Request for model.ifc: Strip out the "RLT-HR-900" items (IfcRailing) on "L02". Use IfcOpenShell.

First a look at what the model holds.

```python
import ifcopenshell
import ifcopenshell.util.element

model = ifcopenshell.open("model.ifc")
print(model.schema)
storey = next(s for s in model.by_type("IfcBuildingStorey") if s.Name == "L02")
railings = [e for e in ifcopenshell.util.element.get_decomposition(storey) if e.is_a("IfcRailing")]
seen = {}
for e in railings:
    element_type = ifcopenshell.util.element.get_type(e)
    name = element_type.Name if element_type not in (None, e) else None
    seen[name] = seen.get(name, 0) + 1
for name, count in sorted(seen.items(), key=str):
    print(count, "x", name)
```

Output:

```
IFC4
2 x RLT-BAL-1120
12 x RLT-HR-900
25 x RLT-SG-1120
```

```python
import ifcopenshell
import ifcopenshell.api.root
import ifcopenshell.util.element

model = ifcopenshell.open("model.ifc")

storey = next(s for s in model.by_type("IfcBuildingStorey") if s.Name == "L02")
railings = [e for e in ifcopenshell.util.element.get_decomposition(storey) if e.is_a("IfcRailing")]
targets = [e for e in railings if (t := ifcopenshell.util.element.get_type(e)) not in (None, e) and t.Name == "RLT-HR-900"]

for e in targets:
    ifcopenshell.api.root.remove_product(model, product=e)
print(len(targets), "removed")

model.write("model_v2.ifc")
```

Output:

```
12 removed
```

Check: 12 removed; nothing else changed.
